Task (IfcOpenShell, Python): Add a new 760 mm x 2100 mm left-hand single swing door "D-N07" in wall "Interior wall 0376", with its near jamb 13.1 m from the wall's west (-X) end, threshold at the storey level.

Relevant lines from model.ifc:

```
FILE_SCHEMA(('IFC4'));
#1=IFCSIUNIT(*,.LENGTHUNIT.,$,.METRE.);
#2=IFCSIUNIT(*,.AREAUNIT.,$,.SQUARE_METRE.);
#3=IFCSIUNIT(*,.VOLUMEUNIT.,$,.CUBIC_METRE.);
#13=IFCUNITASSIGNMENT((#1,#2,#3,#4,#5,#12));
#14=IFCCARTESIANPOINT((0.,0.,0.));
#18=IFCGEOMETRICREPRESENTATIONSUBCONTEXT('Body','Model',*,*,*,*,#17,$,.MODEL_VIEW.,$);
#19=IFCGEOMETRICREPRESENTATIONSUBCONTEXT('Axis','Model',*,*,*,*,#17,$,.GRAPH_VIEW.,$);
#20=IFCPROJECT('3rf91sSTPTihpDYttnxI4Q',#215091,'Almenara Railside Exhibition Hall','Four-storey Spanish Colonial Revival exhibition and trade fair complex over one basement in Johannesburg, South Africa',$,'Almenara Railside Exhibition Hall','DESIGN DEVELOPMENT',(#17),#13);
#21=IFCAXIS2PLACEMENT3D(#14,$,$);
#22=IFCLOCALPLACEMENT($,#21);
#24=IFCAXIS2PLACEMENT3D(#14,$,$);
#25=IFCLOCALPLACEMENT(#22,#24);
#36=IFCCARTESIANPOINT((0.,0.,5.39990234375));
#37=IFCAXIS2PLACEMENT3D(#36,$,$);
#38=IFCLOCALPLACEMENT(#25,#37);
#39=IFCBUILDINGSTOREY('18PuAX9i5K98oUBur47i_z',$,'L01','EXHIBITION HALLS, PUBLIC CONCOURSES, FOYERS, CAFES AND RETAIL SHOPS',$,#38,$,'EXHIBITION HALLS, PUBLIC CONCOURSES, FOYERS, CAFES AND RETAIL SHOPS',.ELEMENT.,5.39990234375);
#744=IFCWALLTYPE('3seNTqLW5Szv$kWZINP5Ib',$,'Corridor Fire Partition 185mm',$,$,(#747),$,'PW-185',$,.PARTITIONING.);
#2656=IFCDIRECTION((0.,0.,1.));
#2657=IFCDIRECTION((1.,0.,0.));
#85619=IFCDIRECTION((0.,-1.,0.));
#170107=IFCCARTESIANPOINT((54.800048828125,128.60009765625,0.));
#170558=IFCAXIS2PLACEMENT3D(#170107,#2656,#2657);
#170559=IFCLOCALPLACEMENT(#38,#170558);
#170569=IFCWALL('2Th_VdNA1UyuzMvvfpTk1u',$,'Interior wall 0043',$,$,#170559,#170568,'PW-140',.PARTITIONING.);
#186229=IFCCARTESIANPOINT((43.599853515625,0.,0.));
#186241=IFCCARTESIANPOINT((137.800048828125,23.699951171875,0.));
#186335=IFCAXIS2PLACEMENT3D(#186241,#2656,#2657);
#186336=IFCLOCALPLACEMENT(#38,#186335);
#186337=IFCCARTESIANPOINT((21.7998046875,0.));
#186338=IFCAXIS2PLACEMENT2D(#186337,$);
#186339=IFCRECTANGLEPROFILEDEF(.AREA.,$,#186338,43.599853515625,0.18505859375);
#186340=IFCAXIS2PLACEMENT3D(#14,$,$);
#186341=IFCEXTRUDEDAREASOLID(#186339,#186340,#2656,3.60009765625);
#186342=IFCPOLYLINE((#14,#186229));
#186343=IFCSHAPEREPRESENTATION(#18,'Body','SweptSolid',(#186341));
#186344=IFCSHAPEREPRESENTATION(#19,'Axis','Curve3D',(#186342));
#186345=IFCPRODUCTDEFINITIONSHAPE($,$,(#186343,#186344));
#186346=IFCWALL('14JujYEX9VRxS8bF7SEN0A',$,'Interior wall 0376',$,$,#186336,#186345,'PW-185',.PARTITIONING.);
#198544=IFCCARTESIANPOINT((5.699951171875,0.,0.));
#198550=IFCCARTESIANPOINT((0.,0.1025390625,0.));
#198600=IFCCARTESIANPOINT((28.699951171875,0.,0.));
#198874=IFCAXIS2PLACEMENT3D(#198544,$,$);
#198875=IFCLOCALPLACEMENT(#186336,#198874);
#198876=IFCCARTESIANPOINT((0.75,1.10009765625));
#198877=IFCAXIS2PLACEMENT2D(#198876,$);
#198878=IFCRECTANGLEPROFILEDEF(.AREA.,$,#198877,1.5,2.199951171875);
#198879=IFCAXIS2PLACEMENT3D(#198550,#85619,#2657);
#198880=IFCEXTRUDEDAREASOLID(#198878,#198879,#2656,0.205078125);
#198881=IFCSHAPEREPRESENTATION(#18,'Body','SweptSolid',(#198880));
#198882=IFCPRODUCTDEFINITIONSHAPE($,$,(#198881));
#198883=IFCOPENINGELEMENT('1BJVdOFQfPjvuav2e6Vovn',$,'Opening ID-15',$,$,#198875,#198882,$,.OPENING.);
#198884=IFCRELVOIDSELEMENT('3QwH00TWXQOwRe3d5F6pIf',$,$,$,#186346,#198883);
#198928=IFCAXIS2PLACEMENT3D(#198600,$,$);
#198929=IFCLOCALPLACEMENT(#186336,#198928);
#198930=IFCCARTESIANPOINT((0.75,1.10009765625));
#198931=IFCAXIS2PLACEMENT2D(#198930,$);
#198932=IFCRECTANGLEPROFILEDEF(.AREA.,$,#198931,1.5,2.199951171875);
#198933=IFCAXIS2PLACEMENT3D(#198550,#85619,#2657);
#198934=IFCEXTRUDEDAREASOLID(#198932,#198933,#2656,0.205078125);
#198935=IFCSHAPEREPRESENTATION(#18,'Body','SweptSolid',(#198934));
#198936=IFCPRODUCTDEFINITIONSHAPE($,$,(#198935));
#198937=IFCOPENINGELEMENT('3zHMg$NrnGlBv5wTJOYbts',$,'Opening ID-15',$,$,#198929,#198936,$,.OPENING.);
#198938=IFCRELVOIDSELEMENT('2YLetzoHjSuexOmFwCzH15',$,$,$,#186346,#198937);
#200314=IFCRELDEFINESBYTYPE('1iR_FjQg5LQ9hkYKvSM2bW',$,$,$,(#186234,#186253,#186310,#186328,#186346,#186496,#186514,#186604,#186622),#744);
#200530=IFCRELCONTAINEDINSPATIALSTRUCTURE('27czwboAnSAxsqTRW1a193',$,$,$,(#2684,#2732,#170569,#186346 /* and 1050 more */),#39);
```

```python
import numpy as np
import ifcopenshell
import ifcopenshell.api.feature
import ifcopenshell.api.geometry
import ifcopenshell.api.root
import ifcopenshell.api.spatial
import ifcopenshell.geom
import ifcopenshell.util.element
import ifcopenshell.util.placement
import ifcopenshell.util.representation
import ifcopenshell.util.shape
import ifcopenshell.util.unit

model = ifcopenshell.open("model.ifc")
unit_scale = ifcopenshell.util.unit.calculate_unit_scale(model)
settings = ifcopenshell.geom.settings()


def volume(element):
    """Net volume in cubic metres, openings subtracted."""
    shape = ifcopenshell.geom.create_shape(settings, element)
    return ifcopenshell.util.shape.get_volume(shape.geometry)


wall = model.by_guid("14JujYEX9VRxS8bF7SEN0A")
storey = ifcopenshell.util.element.get_container(wall, ifc_class="IfcBuildingStorey")
context = ifcopenshell.util.representation.get_context(model, "Model", "Body", "MODEL_VIEW")
before = volume(wall)

width, height, from_end, sill = 0.76, 2.1, 13.1, 0.0  # metres

# The wall runs along its own X axis, and the end named is its -X end.
wall_shape = ifcopenshell.geom.create_shape(settings, wall)
x, y, z = ifcopenshell.util.shape.get_vertices(wall_shape.geometry).T
start = x.min() + from_end
face, thickness = float(y.min()), float(y.max() - y.min())
wall_matrix = ifcopenshell.util.placement.get_local_placement(wall.ObjectPlacement)
level = ifcopenshell.util.placement.get_local_placement(storey.ObjectPlacement)[2, 3]


def in_wall(x, y):
    """Placement at x, y metres in the wall's axes, at sill height."""
    matrix = wall_matrix.copy()
    matrix[:, 3] = wall_matrix @ np.array([x / unit_scale, y / unit_scale, 0.0, 1.0])
    matrix[2, 3] = level + sill / unit_scale
    return matrix


# Opening: a box that overshoots both wall faces by 50 mm.
opening = ifcopenshell.api.root.create_entity(model, ifc_class="IfcOpeningElement", predefined_type="OPENING")
box = ifcopenshell.api.geometry.add_wall_representation(
    model, context=context, length=width, height=height, thickness=thickness + 0.1
)
ifcopenshell.api.geometry.assign_representation(model, product=opening, representation=box)
ifcopenshell.api.geometry.edit_object_placement(model, product=opening, matrix=in_wall(start, face - 0.05), is_si=False)
ifcopenshell.api.feature.add_feature(model, feature=opening, element=wall)

door = ifcopenshell.api.root.create_entity(model, ifc_class="IfcDoor", name="D-N07", predefined_type="DOOR")
door.OverallWidth, door.OverallHeight = width / unit_scale, height / unit_scale
door.OperationType = "SINGLE_SWING_LEFT"
body = ifcopenshell.api.geometry.add_door_representation(
    model,
    context=context,
    overall_width=door.OverallWidth,
    overall_height=door.OverallHeight,
    operation_type="SINGLE_SWING_LEFT",
    lining_properties={"LiningDepth": thickness / unit_scale, "ThresholdDepth": thickness / unit_scale},
)
ifcopenshell.api.geometry.assign_representation(model, product=door, representation=body)
ifcopenshell.api.spatial.assign_container(model, products=[door], relating_structure=storey)
ifcopenshell.api.feature.add_filling(model, opening=opening, element=door)

# The lining spans the wall, so the door starts at the wall face.
ifcopenshell.api.geometry.edit_object_placement(model, product=door, matrix=in_wall(start, face), is_si=False)

after = volume(wall)

print(f"wall volume {before:.3f} -> {after:.3f} m3")

model.write("model_updated.ifc")
```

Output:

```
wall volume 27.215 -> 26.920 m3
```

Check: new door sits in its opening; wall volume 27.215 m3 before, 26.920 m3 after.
